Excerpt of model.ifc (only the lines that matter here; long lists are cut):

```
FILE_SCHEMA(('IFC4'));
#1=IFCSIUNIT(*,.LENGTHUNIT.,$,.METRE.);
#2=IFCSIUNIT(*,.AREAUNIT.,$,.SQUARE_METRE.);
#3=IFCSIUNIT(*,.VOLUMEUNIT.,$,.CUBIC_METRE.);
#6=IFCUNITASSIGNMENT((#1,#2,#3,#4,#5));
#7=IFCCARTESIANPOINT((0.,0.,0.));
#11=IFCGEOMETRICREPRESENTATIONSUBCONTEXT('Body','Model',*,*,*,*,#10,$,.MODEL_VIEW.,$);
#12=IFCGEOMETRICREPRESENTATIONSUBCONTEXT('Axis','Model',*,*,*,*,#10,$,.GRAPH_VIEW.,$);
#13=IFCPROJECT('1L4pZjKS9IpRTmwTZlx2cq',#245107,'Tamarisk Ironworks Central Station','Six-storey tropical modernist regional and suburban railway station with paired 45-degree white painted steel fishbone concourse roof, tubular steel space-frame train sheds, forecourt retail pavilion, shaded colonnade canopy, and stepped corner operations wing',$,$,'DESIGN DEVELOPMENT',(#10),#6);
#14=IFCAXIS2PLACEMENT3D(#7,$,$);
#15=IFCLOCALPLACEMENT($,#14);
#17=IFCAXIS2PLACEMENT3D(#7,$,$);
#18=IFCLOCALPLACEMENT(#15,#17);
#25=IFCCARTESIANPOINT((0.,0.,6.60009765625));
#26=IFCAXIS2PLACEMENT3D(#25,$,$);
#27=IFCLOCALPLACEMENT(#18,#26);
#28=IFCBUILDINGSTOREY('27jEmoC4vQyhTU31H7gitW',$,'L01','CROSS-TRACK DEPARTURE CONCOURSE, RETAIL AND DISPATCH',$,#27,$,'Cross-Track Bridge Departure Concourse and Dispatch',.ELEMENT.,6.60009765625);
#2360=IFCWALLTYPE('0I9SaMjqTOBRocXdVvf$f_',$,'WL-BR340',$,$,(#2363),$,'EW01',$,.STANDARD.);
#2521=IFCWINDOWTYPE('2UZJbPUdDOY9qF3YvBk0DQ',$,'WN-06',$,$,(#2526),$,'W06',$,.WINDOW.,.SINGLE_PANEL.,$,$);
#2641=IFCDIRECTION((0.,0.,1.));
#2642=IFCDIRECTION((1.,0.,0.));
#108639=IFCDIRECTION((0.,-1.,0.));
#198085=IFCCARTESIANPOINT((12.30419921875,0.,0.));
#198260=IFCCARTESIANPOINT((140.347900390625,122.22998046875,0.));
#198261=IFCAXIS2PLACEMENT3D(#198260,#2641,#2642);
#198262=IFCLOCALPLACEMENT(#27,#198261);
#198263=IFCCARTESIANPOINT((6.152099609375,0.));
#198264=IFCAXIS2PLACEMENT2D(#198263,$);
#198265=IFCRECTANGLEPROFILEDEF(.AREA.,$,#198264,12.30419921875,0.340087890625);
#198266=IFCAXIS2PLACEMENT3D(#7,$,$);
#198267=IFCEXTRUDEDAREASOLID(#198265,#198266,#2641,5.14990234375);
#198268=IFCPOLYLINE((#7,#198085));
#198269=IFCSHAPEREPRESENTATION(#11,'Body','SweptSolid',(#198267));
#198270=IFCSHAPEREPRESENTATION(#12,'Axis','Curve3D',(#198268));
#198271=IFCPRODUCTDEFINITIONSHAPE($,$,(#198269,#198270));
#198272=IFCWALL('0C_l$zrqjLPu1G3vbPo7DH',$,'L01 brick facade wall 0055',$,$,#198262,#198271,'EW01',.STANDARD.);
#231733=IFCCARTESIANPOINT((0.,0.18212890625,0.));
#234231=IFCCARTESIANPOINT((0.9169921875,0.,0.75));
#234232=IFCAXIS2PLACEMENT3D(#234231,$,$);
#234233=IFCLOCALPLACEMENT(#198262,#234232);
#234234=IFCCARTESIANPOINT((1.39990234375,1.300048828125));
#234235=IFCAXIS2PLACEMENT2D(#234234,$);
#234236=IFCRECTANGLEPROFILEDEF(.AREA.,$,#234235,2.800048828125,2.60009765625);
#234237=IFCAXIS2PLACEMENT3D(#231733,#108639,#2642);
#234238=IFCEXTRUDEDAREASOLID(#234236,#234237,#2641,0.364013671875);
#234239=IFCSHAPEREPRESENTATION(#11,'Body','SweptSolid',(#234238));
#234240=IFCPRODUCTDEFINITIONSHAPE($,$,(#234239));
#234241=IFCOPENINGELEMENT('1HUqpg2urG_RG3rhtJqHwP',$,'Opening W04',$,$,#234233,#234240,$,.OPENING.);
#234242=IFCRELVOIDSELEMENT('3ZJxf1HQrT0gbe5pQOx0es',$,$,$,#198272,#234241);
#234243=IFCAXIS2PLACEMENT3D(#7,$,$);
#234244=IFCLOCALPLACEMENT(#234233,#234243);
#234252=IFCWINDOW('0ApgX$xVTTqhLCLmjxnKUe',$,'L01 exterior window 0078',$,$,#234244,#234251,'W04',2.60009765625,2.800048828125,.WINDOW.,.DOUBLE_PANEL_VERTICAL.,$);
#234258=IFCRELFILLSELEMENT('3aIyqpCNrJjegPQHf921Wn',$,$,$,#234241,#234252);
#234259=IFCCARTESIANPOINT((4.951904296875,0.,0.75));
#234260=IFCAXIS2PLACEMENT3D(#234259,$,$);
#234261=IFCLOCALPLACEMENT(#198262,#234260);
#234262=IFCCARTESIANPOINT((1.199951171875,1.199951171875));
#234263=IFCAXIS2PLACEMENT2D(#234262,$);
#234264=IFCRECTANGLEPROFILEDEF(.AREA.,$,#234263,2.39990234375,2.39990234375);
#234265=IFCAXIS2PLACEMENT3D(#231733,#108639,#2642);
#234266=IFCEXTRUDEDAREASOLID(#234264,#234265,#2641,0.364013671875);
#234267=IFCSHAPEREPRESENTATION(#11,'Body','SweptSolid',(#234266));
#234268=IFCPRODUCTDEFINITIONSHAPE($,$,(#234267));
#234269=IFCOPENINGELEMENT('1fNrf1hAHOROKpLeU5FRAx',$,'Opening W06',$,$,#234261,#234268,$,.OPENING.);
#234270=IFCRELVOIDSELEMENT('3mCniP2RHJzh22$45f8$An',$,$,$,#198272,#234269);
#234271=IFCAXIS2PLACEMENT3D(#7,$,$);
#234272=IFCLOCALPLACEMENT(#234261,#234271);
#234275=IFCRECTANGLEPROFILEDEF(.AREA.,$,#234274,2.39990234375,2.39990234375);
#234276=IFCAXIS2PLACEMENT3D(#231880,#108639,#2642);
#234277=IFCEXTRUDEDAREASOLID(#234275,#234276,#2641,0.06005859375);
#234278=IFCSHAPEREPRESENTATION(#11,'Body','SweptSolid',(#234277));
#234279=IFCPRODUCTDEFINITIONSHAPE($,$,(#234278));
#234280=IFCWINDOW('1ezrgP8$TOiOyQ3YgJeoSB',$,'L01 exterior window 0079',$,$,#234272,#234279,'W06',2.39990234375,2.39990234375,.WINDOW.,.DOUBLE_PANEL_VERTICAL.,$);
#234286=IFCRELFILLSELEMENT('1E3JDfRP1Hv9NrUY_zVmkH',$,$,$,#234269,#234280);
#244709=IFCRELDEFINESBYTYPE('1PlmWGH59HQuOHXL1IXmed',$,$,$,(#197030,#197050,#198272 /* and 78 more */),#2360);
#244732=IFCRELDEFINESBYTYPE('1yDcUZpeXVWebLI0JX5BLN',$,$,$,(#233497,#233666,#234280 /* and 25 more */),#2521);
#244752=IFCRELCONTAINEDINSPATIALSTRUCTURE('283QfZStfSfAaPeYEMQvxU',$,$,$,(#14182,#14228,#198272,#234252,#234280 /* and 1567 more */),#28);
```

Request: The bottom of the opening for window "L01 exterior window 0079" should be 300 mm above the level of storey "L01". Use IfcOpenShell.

```python
import numpy as np
import ifcopenshell
import ifcopenshell.api.geometry
import ifcopenshell.geom
import ifcopenshell.util.element
import ifcopenshell.util.placement
import ifcopenshell.util.shape
import ifcopenshell.util.unit

model = ifcopenshell.open("model.ifc")
unit_scale = ifcopenshell.util.unit.calculate_unit_scale(model)

window = model.by_guid("1ezrgP8$TOiOyQ3YgJeoSB")
opening = window.FillsVoids[0].RelatingOpeningElement
storey = ifcopenshell.util.element.get_container(window, ifc_class="IfcBuildingStorey")
level = ifcopenshell.util.placement.get_local_placement(storey.ObjectPlacement)[2, 3]

# The opening's origin need not be at the sill, so measure its lowest point.
shape = ifcopenshell.geom.create_shape(ifcopenshell.geom.settings(), opening)
bottom = ifcopenshell.util.shape.get_shape_bottom_elevation(shape, shape.geometry) / unit_scale
dz = level + 0.3 - bottom

shift = np.array([0.0, 0.0, dz])
# The window is placed relative to its opening, so it follows when the opening moves.
matrix = ifcopenshell.util.placement.get_local_placement(opening.ObjectPlacement)
matrix[:3, 3] += shift
ifcopenshell.api.geometry.edit_object_placement(
    model, product=opening, matrix=matrix, is_si=False, should_transform_children=True
)

print(f"moved by {dz * unit_scale:+.3f} m")

model.write("model-out.ifc")
```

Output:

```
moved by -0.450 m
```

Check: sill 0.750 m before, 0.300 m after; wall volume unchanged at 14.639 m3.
